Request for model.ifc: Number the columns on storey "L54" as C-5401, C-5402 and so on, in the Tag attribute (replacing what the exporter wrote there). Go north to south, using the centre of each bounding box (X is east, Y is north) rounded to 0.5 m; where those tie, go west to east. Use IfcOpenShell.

First a look at what the model holds.

```python
import ifcopenshell
import ifcopenshell.util.element
import ifcopenshell.util.placement

model = ifcopenshell.open("model.ifc")
print(model.schema)
storey = next(s for s in model.by_type("IfcBuildingStorey") if s.Name == "L54")
columns = [e for e in ifcopenshell.util.element.get_decomposition(storey) if e.is_a("IfcColumn")]
for e in sorted(columns, key=lambda e: e.id()):
    origin = ifcopenshell.util.placement.get_local_placement(e.ObjectPlacement)[:3, 3]
    print(e.id(), e.Tag, e.Name, origin.round(2) + 0.0, sep=" | ")
```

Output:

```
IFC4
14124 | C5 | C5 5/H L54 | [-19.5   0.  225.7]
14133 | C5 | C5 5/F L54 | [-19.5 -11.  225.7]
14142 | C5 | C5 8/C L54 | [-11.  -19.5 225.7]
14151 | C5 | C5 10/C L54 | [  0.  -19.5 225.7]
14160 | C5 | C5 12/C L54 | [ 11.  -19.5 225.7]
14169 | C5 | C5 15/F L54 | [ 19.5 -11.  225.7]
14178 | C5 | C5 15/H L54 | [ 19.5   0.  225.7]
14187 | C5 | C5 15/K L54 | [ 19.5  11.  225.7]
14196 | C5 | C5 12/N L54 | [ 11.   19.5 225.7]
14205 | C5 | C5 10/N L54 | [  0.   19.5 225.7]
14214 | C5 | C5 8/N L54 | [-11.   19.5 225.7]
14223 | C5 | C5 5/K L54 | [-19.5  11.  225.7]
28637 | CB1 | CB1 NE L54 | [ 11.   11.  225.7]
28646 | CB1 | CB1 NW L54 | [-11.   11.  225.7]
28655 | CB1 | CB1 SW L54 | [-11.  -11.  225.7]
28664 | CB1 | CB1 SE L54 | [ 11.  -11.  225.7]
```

```python
import ifcopenshell
import ifcopenshell.geom
import ifcopenshell.util.element
import ifcopenshell.util.shape

model = ifcopenshell.open("model.ifc")
settings = ifcopenshell.geom.settings()
settings.set("use-world-coords", True)


def centre(element):
    shape = ifcopenshell.geom.create_shape(settings, element)
    return ifcopenshell.util.shape.get_bbox_centroid(shape.geometry)


storey = next(s for s in model.by_type("IfcBuildingStorey") if s.Name == "L54")
columns = [e for e in ifcopenshell.util.element.get_decomposition(storey) if e.is_a("IfcColumn")]

# Insertion points can sit at a corner or the storey origin, so sort by the geometry (in metres).
centres = {e: centre(e) for e in columns}
columns.sort(key=lambda e: (-round(centres[e][1] / 0.5), centres[e][0]))

for i, e in enumerate(columns, start=1):
    number = f"C-54{i:02d}"
    e.Tag = number
    print(e.id(), number)

model.write("model-out.ifc")
```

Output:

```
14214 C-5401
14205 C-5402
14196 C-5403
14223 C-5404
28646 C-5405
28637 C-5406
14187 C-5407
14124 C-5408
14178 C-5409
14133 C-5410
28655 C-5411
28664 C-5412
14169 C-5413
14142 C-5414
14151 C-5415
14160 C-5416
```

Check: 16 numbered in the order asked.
